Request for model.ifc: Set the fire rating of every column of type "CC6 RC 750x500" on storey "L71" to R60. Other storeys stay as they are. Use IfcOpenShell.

First a look at what the model holds.

```python
import ifcopenshell
import ifcopenshell.util.element

model = ifcopenshell.open("model.ifc")
print(model.schema)
storey = next(s for s in model.by_type("IfcBuildingStorey") if s.Name == "L71")
columns = [e for e in ifcopenshell.util.element.get_decomposition(storey) if e.is_a("IfcColumn")]
seen = {}
for e in columns:
    element_type = ifcopenshell.util.element.get_type(e)
    key = (element_type.Name if element_type != e and element_type else None, ifcopenshell.util.element.get_pset(e, "Pset_ColumnCommon", "FireRating"))
    seen[key] = seen.get(key, 0) + 1
for (name, value), count in sorted(seen.items(), key=str):
    print(count, "x", name, "|", value)
```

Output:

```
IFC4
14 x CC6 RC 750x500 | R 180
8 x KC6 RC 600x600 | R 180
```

```python
import ifcopenshell
import ifcopenshell.api.pset
import ifcopenshell.util.element

model = ifcopenshell.open("model.ifc")

storey = next(s for s in model.by_type("IfcBuildingStorey") if s.Name == "L71")
columns = [e for e in ifcopenshell.util.element.get_decomposition(storey) if e.is_a("IfcColumn")]

count = 0
for e in columns:
    element_type = ifcopenshell.util.element.get_type(e)
    if element_type in (None, e) or element_type.Name != "CC6 RC 750x500":
        continue
    found = ifcopenshell.util.element.get_pset(e, "Pset_ColumnCommon", should_inherit=False)
    if found:
        pset = model.by_id(found["id"])
        if len(ifcopenshell.util.element.get_elements_by_pset(pset)) > 1:
            pset = ifcopenshell.api.pset.unshare_pset(model, products=[e], pset=pset)[0]
    else:
        pset = ifcopenshell.api.pset.add_pset(model, product=e, name="Pset_ColumnCommon")
    ifcopenshell.api.pset.edit_pset(model, pset=pset, properties={"FireRating": "R60"})
    count += 1

print(count, "columns updated")

model.write("model_v2.ifc")
```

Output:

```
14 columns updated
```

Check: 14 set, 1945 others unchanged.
